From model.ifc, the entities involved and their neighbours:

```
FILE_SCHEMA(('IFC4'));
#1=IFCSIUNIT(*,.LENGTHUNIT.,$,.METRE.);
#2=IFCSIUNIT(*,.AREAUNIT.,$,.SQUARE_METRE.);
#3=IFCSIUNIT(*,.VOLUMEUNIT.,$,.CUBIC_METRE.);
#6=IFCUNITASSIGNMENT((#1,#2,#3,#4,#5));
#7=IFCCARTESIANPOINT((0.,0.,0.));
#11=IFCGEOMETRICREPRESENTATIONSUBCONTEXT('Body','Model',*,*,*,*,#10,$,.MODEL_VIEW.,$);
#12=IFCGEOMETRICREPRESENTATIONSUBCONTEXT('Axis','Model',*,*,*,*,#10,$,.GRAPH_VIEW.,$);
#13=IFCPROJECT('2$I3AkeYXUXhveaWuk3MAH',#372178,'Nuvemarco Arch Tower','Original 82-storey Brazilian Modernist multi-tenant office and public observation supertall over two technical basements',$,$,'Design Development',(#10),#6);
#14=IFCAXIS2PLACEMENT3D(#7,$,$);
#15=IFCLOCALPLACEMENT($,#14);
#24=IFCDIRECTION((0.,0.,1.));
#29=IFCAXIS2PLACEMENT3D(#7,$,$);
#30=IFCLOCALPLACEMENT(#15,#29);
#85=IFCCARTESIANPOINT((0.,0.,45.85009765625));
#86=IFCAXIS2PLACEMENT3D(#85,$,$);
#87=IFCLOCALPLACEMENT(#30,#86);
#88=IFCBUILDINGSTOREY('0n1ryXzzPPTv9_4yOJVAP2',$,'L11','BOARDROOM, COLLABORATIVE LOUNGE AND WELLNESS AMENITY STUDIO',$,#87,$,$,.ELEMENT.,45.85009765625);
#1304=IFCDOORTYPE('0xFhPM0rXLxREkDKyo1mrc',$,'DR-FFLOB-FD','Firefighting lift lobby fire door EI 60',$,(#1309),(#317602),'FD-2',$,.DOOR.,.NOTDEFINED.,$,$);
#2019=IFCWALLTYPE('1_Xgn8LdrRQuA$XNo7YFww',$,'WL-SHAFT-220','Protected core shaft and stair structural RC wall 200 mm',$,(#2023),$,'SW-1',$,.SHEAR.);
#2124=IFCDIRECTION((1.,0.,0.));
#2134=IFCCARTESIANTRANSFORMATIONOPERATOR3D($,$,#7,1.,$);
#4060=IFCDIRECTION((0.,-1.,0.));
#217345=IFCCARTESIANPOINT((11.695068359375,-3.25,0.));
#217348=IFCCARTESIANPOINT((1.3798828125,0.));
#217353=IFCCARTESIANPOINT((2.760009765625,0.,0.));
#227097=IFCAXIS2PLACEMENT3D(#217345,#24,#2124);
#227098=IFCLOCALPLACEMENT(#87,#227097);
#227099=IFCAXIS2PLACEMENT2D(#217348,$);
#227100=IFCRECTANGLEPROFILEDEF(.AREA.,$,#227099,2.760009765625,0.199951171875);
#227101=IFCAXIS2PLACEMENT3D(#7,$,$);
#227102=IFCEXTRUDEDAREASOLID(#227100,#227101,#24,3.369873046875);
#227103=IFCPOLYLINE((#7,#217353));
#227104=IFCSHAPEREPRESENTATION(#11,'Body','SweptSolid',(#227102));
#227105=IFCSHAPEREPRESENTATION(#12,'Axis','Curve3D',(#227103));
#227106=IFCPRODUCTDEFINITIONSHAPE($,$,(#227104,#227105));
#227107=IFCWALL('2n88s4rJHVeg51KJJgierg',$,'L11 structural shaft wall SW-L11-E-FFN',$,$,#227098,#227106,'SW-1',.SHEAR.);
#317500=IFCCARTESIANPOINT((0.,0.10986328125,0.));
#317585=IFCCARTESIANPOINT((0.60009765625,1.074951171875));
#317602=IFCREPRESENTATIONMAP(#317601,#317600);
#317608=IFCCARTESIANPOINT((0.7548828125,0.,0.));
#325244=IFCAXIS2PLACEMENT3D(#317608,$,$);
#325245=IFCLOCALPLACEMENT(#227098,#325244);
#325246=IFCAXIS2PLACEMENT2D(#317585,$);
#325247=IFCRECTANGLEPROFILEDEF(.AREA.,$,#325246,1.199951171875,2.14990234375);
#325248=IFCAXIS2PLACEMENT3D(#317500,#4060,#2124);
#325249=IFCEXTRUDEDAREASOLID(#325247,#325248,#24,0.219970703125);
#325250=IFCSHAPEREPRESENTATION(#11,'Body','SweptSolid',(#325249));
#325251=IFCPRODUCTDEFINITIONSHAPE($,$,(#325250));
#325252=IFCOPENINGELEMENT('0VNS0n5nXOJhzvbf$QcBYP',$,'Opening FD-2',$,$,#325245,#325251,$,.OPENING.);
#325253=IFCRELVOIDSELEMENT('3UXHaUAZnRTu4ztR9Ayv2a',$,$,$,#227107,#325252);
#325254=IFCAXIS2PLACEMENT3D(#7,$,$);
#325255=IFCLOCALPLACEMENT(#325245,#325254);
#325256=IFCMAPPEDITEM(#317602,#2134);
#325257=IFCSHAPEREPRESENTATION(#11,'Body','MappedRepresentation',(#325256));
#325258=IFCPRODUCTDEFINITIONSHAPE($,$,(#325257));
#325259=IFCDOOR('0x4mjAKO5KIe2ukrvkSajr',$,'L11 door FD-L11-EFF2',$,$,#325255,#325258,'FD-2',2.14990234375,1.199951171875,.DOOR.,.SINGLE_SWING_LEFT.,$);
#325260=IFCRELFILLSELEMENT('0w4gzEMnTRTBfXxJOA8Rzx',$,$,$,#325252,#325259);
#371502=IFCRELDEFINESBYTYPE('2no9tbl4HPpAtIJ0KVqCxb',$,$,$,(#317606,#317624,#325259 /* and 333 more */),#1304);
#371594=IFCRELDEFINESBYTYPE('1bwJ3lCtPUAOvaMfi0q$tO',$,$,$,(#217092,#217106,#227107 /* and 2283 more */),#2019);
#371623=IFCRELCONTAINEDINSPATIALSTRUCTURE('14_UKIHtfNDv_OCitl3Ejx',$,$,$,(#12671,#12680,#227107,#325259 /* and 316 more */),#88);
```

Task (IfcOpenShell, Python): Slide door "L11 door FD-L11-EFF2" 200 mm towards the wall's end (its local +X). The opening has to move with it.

```python
import ifcopenshell
import ifcopenshell.api.geometry
import ifcopenshell.util.placement
import ifcopenshell.util.unit

model = ifcopenshell.open("model.ifc")
unit_scale = ifcopenshell.util.unit.calculate_unit_scale(model)

door = model.by_guid("0x4mjAKO5KIe2ukrvkSajr")
opening = door.FillsVoids[0].RelatingOpeningElement
wall = opening.VoidsElements[0].RelatingBuildingElement

wall_matrix = ifcopenshell.util.placement.get_local_placement(wall.ObjectPlacement)
shift = wall_matrix[:3, 0] * 0.2 / unit_scale
before = ifcopenshell.util.placement.get_local_placement(door.ObjectPlacement)[:3, 3].copy()

# The door is placed relative to its opening, so it follows when the opening moves.
matrix = ifcopenshell.util.placement.get_local_placement(opening.ObjectPlacement)
matrix[:3, 3] += shift
ifcopenshell.api.geometry.edit_object_placement(
    model, product=opening, matrix=matrix, is_si=False, should_transform_children=True
)

after = ifcopenshell.util.placement.get_local_placement(door.ObjectPlacement)[:3, 3]
print("door moved by", (after - before).round(3) + 0.0)

model.write("model_updated.ifc")
```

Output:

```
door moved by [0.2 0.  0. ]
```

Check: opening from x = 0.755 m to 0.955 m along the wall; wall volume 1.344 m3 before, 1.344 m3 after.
